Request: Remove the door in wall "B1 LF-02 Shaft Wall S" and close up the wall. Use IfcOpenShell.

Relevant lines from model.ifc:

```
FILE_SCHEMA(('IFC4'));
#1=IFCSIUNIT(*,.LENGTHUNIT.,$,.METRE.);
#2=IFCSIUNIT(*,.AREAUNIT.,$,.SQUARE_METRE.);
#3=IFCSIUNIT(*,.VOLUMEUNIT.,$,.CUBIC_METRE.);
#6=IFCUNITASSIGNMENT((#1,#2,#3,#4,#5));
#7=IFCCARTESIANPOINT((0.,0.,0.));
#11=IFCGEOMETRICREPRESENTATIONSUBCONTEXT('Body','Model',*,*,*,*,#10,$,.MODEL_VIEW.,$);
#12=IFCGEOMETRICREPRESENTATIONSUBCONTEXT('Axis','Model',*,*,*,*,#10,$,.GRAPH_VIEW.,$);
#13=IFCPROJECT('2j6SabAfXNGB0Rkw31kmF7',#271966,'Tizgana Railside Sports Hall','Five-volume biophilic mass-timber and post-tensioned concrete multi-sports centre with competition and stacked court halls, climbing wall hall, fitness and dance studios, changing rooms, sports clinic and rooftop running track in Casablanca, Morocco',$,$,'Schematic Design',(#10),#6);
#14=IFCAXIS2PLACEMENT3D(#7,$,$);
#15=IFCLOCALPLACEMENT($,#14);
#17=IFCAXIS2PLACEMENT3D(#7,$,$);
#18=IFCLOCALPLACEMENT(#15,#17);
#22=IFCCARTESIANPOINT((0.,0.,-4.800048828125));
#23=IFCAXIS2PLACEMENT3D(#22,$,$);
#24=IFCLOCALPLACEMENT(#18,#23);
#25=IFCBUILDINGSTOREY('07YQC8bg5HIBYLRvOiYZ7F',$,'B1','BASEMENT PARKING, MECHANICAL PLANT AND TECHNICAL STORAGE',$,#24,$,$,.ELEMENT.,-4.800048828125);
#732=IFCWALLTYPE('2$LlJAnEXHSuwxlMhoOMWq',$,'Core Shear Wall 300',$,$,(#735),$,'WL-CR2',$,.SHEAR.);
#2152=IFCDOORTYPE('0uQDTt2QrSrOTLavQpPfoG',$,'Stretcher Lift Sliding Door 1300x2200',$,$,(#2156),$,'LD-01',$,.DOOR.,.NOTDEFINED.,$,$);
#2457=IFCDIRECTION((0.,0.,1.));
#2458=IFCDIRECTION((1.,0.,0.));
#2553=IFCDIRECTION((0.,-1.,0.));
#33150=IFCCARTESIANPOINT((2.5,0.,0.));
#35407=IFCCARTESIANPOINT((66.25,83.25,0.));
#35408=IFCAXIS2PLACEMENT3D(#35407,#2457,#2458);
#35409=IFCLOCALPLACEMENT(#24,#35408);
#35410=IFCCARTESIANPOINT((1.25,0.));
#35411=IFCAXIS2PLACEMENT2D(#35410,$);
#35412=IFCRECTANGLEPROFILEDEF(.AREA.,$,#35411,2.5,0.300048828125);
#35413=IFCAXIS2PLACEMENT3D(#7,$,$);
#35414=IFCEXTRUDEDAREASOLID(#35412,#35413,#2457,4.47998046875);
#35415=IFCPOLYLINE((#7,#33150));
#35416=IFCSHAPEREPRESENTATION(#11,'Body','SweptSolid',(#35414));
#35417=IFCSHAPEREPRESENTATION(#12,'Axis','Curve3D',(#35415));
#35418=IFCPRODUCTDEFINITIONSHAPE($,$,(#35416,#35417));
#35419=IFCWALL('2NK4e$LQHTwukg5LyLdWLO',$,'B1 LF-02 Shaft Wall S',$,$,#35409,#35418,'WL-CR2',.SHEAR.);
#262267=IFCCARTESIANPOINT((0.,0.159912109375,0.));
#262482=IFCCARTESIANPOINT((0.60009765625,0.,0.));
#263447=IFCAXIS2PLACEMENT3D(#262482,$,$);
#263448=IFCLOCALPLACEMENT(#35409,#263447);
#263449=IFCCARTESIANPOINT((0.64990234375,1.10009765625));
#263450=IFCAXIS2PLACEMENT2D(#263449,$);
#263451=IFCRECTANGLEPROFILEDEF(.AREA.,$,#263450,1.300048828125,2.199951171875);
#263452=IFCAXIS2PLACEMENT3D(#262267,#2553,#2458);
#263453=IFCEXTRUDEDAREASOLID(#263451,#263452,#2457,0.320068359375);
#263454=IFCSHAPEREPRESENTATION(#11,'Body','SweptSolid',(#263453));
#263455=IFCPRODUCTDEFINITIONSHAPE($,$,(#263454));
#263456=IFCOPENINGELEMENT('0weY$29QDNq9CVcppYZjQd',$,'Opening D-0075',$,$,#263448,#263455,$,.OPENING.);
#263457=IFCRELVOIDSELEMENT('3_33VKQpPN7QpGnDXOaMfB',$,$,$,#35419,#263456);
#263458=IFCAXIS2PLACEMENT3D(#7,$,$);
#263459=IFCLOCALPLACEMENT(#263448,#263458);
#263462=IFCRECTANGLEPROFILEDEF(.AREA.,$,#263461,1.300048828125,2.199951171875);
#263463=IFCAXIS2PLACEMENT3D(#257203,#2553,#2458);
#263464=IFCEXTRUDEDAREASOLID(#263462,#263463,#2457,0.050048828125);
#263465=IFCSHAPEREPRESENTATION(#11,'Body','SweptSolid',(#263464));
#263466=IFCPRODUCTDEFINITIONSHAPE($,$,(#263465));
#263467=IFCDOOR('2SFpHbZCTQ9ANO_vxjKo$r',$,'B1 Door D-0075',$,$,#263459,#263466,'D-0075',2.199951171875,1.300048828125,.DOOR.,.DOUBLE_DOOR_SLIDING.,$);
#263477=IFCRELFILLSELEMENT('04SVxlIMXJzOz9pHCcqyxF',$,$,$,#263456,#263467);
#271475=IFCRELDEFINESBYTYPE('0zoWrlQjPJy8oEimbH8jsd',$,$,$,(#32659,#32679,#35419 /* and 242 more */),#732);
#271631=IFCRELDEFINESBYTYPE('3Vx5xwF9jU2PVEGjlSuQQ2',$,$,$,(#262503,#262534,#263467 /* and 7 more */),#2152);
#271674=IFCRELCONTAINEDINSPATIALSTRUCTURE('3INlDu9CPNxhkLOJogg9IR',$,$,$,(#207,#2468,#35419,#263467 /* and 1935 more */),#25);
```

```python
import ifcopenshell
import ifcopenshell.api.feature
import ifcopenshell.api.root
import ifcopenshell.geom
import ifcopenshell.util.shape

model = ifcopenshell.open("model.ifc")
settings = ifcopenshell.geom.settings()


def volume(element):
    """Net volume in cubic metres, openings subtracted."""
    shape = ifcopenshell.geom.create_shape(settings, element)
    return ifcopenshell.util.shape.get_volume(shape.geometry)


door = model.by_guid("2SFpHbZCTQ9ANO_vxjKo$r")
opening = door.FillsVoids[0].RelatingOpeningElement
wall = opening.VoidsElements[0].RelatingBuildingElement
before = volume(wall)

ifcopenshell.api.root.remove_product(model, product=door)
ifcopenshell.api.feature.remove_feature(model, feature=opening)

after = volume(wall)

print(f"wall volume {before:.3f} -> {after:.3f} m3")

model.write("model_updated.ifc")
```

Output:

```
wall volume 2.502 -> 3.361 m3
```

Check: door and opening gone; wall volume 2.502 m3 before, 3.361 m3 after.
